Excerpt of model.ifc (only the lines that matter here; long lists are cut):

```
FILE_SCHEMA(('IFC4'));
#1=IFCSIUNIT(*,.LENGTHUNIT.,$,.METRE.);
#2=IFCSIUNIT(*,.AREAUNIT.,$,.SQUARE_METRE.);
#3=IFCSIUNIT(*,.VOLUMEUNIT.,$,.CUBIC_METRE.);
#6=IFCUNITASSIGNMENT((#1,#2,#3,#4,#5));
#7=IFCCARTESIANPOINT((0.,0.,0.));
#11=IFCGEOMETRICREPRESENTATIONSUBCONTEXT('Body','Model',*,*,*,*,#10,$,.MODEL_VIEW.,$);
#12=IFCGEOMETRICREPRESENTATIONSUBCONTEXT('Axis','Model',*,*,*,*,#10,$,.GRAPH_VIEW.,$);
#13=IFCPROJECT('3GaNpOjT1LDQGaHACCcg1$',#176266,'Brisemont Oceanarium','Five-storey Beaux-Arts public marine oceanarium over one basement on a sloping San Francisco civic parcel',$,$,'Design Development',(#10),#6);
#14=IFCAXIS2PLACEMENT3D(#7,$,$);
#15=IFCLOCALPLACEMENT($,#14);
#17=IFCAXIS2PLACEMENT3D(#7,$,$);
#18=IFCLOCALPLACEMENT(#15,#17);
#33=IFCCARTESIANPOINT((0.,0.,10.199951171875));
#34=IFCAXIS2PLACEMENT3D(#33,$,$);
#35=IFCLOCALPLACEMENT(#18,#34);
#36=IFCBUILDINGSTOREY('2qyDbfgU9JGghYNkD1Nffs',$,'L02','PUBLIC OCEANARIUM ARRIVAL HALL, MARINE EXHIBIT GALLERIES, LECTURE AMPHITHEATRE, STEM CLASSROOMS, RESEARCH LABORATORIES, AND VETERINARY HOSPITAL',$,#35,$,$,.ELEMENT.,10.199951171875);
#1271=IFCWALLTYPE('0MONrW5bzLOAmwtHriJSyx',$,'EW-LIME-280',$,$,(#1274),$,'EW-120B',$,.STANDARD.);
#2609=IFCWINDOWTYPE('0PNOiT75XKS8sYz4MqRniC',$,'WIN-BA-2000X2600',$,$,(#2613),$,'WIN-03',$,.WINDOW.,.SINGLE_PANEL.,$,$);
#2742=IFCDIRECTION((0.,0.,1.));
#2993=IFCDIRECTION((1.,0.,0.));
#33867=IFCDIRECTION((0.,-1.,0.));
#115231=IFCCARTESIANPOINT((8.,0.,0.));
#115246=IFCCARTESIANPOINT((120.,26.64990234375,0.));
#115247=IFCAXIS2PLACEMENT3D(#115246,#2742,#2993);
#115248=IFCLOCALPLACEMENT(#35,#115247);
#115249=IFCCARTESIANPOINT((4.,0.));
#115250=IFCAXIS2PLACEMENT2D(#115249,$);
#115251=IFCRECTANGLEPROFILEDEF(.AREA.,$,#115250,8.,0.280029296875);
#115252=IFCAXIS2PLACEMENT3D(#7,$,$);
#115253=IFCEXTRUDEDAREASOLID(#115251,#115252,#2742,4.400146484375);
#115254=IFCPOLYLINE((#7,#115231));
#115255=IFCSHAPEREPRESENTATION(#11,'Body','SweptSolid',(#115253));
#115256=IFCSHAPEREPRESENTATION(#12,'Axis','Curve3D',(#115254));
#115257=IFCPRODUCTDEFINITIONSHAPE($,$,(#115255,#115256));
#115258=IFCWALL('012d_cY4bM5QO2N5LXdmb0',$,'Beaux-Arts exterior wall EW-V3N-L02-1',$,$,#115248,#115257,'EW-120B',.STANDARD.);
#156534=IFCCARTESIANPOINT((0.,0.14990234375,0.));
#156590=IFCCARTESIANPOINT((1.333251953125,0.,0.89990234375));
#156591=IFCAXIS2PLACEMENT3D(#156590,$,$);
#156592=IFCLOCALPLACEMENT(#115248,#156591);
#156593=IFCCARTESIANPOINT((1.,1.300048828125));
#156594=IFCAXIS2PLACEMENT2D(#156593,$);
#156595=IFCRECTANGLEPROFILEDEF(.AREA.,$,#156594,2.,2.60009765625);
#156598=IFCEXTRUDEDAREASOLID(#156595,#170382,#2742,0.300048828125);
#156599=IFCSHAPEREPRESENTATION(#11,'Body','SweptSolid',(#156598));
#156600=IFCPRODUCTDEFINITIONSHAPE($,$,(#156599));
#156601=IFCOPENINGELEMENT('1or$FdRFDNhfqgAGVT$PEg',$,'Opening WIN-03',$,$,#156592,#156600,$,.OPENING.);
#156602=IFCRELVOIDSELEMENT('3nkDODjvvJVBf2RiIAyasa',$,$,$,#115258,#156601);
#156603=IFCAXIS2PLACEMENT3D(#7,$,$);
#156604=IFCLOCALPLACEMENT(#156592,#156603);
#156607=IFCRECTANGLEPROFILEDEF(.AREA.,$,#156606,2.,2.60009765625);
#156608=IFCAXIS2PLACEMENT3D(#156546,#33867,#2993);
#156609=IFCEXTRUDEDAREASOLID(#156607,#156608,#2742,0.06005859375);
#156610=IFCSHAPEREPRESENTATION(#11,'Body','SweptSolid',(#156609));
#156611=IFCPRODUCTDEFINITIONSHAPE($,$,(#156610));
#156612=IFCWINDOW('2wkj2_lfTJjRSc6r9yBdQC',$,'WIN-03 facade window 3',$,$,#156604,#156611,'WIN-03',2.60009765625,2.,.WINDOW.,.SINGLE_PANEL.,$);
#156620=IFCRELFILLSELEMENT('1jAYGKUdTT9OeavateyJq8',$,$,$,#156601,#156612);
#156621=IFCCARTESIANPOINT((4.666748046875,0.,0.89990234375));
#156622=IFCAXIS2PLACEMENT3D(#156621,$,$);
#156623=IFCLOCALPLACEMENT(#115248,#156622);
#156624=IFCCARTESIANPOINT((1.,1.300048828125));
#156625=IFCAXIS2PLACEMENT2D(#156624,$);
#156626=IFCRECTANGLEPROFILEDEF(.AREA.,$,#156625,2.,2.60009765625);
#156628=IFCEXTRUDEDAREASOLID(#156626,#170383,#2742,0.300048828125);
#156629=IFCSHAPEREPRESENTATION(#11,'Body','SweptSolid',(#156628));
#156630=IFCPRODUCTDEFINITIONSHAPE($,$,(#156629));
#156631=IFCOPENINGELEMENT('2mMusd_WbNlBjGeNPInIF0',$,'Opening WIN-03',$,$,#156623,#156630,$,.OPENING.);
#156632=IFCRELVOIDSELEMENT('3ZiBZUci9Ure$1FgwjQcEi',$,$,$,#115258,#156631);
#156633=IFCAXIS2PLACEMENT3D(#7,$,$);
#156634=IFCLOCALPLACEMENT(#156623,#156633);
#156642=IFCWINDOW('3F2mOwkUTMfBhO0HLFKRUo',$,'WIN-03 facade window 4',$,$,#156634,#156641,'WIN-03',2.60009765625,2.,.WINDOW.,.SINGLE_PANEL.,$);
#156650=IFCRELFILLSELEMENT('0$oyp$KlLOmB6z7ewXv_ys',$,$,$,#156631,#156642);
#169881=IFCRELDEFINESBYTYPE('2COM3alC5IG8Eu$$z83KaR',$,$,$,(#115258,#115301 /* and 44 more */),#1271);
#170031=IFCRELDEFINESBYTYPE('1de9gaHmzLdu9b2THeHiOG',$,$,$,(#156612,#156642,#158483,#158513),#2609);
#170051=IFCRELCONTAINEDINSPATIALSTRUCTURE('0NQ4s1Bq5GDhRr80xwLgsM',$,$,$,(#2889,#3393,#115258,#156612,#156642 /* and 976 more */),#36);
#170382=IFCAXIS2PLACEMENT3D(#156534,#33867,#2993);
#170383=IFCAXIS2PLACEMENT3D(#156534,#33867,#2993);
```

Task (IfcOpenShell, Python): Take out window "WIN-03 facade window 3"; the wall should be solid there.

```python
import ifcopenshell
import ifcopenshell.api.feature
import ifcopenshell.api.root
import ifcopenshell.geom
import ifcopenshell.util.shape

model = ifcopenshell.open("model.ifc")
settings = ifcopenshell.geom.settings()


def volume(element):
    """Net volume in cubic metres, openings subtracted."""
    shape = ifcopenshell.geom.create_shape(settings, element)
    return ifcopenshell.util.shape.get_volume(shape.geometry)


window = model.by_id(156612)
opening = window.FillsVoids[0].RelatingOpeningElement
wall = opening.VoidsElements[0].RelatingBuildingElement
before = volume(wall)

ifcopenshell.api.root.remove_product(model, product=window)
ifcopenshell.api.feature.remove_feature(model, feature=opening)

after = volume(wall)

print(f"wall volume {before:.3f} -> {after:.3f} m3")

model.write("model_updated.ifc")
```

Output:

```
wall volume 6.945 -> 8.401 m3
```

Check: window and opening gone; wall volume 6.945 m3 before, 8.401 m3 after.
